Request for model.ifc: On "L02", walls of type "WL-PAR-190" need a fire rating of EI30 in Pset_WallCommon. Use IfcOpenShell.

First a look at what the model holds.

```python
import ifcopenshell
import ifcopenshell.util.element

model = ifcopenshell.open("model.ifc")
print(model.schema)
storey = next(s for s in model.by_type("IfcBuildingStorey") if s.Name == "L02")
walls = [e for e in ifcopenshell.util.element.get_decomposition(storey) if e.is_a("IfcWall")]
seen = {}
for e in walls:
    element_type = ifcopenshell.util.element.get_type(e)
    key = (element_type.Name if element_type != e and element_type else None, ifcopenshell.util.element.get_pset(e, "Pset_WallCommon", "FireRating"))
    seen[key] = seen.get(key, 0) + 1
for (name, value), count in sorted(seen.items(), key=str):
    print(count, "x", name, "|", value)
```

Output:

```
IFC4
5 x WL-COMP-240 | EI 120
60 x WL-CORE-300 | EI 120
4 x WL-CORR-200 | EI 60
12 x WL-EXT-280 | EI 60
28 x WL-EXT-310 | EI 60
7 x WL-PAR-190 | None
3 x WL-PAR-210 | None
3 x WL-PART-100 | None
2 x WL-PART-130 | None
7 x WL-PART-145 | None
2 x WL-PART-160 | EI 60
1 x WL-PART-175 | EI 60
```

```python
import ifcopenshell
import ifcopenshell.api.pset
import ifcopenshell.util.element

model = ifcopenshell.open("model.ifc")

storey = next(s for s in model.by_type("IfcBuildingStorey") if s.Name == "L02")
walls = [e for e in ifcopenshell.util.element.get_decomposition(storey) if e.is_a("IfcWall")]

count = 0
for e in walls:
    element_type = ifcopenshell.util.element.get_type(e)
    if element_type in (None, e) or element_type.Name != "WL-PAR-190":
        continue
    # add_pset returns the element's existing set when there is one.
    pset = ifcopenshell.api.pset.add_pset(model, product=e, name="Pset_WallCommon")
    ifcopenshell.api.pset.edit_pset(model, pset=pset, properties={"FireRating": "EI30"})
    count += 1

print(count, "walls updated")

model.write("model_v2.ifc")
```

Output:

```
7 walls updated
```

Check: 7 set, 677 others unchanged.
